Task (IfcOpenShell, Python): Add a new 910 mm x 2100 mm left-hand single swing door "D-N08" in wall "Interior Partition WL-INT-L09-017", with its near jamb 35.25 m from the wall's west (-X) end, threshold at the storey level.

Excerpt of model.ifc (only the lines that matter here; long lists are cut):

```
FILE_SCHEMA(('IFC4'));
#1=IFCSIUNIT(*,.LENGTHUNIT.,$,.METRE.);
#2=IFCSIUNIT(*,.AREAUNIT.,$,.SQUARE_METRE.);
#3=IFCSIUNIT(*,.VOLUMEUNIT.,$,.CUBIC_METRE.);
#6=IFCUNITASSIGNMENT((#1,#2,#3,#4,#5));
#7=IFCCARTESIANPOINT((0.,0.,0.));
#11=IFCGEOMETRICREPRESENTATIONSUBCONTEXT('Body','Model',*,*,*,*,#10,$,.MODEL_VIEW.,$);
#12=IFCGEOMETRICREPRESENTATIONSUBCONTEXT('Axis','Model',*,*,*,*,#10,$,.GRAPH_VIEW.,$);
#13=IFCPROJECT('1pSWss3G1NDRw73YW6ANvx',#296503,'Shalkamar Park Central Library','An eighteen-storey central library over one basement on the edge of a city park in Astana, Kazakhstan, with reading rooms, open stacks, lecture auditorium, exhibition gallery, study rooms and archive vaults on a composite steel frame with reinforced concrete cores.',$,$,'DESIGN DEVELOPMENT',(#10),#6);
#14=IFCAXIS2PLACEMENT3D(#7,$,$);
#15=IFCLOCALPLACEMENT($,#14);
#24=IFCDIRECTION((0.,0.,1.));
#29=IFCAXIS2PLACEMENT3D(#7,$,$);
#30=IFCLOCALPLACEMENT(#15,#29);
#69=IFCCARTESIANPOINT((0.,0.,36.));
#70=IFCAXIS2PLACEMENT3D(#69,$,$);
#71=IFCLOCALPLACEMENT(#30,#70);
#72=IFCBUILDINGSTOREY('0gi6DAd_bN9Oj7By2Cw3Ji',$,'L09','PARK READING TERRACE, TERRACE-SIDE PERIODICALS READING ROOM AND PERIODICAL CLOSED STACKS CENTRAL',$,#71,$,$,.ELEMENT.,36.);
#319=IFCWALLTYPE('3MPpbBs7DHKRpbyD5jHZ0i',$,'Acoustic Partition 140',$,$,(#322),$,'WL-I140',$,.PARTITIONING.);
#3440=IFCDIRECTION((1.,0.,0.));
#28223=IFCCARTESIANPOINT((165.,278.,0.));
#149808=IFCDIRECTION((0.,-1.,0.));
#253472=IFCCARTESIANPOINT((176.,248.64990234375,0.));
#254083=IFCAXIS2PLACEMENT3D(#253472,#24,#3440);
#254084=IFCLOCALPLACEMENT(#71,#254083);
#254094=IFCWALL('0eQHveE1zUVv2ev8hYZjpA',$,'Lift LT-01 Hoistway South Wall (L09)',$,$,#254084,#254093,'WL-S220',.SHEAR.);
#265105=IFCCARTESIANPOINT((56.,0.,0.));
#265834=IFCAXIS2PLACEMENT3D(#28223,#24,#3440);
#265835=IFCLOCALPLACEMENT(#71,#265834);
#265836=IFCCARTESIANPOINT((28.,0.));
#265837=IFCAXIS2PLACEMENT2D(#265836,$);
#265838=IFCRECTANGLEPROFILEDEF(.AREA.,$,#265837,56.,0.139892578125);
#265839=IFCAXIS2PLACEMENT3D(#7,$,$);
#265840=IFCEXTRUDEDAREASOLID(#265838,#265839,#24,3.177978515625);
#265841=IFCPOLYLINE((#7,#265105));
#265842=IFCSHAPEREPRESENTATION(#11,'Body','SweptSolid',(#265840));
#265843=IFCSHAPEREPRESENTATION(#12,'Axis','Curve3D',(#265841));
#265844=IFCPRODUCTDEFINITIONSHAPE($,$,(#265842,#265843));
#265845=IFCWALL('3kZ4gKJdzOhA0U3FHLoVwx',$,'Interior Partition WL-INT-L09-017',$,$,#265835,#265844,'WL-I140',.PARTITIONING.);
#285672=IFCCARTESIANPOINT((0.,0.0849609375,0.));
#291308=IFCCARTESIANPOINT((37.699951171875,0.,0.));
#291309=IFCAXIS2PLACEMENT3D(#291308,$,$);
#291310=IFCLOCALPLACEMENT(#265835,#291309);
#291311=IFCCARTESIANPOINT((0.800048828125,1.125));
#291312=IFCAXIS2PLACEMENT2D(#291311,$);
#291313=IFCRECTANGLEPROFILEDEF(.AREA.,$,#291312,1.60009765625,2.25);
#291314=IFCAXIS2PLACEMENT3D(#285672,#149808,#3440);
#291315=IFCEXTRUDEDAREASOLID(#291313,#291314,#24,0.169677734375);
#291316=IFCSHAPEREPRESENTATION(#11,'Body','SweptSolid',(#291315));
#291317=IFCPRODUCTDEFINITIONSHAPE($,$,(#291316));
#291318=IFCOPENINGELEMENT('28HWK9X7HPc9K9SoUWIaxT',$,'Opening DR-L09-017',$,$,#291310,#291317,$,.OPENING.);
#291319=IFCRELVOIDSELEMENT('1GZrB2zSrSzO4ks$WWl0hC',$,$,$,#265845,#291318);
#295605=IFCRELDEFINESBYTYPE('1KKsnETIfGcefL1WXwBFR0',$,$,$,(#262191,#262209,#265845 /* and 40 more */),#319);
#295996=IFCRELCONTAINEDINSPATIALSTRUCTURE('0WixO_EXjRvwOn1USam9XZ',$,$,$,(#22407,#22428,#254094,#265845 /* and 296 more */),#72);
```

```python
import numpy as np
import ifcopenshell
import ifcopenshell.api.feature
import ifcopenshell.api.geometry
import ifcopenshell.api.root
import ifcopenshell.api.spatial
import ifcopenshell.geom
import ifcopenshell.util.element
import ifcopenshell.util.placement
import ifcopenshell.util.representation
import ifcopenshell.util.shape
import ifcopenshell.util.unit

model = ifcopenshell.open("model.ifc")
unit_scale = ifcopenshell.util.unit.calculate_unit_scale(model)
settings = ifcopenshell.geom.settings()


def volume(element):
    """Net volume in cubic metres, openings subtracted."""
    shape = ifcopenshell.geom.create_shape(settings, element)
    return ifcopenshell.util.shape.get_volume(shape.geometry)


wall = model.by_guid("3kZ4gKJdzOhA0U3FHLoVwx")
storey = ifcopenshell.util.element.get_container(wall, ifc_class="IfcBuildingStorey")
context = ifcopenshell.util.representation.get_context(model, "Model", "Body", "MODEL_VIEW")
before = volume(wall)

width, height, from_end, sill = 0.91, 2.1, 35.25, 0.0  # metres

# The wall runs along its own X axis, and the end named is its -X end.
wall_shape = ifcopenshell.geom.create_shape(settings, wall)
x, y, z = ifcopenshell.util.shape.get_vertices(wall_shape.geometry).T
start = x.min() + from_end
face, thickness = float(y.min()), float(y.max() - y.min())
wall_matrix = ifcopenshell.util.placement.get_local_placement(wall.ObjectPlacement)
level = ifcopenshell.util.placement.get_local_placement(storey.ObjectPlacement)[2, 3]


def in_wall(x, y):
    """Placement at x, y metres in the wall's axes, at sill height."""
    matrix = wall_matrix.copy()
    matrix[:, 3] = wall_matrix @ np.array([x / unit_scale, y / unit_scale, 0.0, 1.0])
    matrix[2, 3] = level + sill / unit_scale
    return matrix


# Opening: a box that overshoots both wall faces by 50 mm.
opening = ifcopenshell.api.root.create_entity(model, ifc_class="IfcOpeningElement", predefined_type="OPENING")
box = ifcopenshell.api.geometry.add_wall_representation(
    model, context=context, length=width, height=height, thickness=thickness + 0.1
)
ifcopenshell.api.geometry.assign_representation(model, product=opening, representation=box)
ifcopenshell.api.geometry.edit_object_placement(model, product=opening, matrix=in_wall(start, face - 0.05), is_si=False)
ifcopenshell.api.feature.add_feature(model, feature=opening, element=wall)

door = ifcopenshell.api.root.create_entity(model, ifc_class="IfcDoor", name="D-N08", predefined_type="DOOR")
door.OverallWidth, door.OverallHeight = width / unit_scale, height / unit_scale
door.OperationType = "SINGLE_SWING_LEFT"
body = ifcopenshell.api.geometry.add_door_representation(
    model,
    context=context,
    overall_width=door.OverallWidth,
    overall_height=door.OverallHeight,
    operation_type="SINGLE_SWING_LEFT",
    lining_properties={"LiningDepth": thickness / unit_scale, "ThresholdDepth": thickness / unit_scale},
)
ifcopenshell.api.geometry.assign_representation(model, product=door, representation=body)
ifcopenshell.api.spatial.assign_container(model, products=[door], relating_structure=storey)
ifcopenshell.api.feature.add_filling(model, opening=opening, element=door)

# The lining spans the wall, so the door starts at the wall face.
ifcopenshell.api.geometry.edit_object_placement(model, product=door, matrix=in_wall(start, face), is_si=False)

after = volume(wall)

print(f"wall volume {before:.3f} -> {after:.3f} m3")

model.write("model_rev.ifc")
```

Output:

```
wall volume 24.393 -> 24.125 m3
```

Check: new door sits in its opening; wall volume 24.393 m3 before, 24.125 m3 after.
